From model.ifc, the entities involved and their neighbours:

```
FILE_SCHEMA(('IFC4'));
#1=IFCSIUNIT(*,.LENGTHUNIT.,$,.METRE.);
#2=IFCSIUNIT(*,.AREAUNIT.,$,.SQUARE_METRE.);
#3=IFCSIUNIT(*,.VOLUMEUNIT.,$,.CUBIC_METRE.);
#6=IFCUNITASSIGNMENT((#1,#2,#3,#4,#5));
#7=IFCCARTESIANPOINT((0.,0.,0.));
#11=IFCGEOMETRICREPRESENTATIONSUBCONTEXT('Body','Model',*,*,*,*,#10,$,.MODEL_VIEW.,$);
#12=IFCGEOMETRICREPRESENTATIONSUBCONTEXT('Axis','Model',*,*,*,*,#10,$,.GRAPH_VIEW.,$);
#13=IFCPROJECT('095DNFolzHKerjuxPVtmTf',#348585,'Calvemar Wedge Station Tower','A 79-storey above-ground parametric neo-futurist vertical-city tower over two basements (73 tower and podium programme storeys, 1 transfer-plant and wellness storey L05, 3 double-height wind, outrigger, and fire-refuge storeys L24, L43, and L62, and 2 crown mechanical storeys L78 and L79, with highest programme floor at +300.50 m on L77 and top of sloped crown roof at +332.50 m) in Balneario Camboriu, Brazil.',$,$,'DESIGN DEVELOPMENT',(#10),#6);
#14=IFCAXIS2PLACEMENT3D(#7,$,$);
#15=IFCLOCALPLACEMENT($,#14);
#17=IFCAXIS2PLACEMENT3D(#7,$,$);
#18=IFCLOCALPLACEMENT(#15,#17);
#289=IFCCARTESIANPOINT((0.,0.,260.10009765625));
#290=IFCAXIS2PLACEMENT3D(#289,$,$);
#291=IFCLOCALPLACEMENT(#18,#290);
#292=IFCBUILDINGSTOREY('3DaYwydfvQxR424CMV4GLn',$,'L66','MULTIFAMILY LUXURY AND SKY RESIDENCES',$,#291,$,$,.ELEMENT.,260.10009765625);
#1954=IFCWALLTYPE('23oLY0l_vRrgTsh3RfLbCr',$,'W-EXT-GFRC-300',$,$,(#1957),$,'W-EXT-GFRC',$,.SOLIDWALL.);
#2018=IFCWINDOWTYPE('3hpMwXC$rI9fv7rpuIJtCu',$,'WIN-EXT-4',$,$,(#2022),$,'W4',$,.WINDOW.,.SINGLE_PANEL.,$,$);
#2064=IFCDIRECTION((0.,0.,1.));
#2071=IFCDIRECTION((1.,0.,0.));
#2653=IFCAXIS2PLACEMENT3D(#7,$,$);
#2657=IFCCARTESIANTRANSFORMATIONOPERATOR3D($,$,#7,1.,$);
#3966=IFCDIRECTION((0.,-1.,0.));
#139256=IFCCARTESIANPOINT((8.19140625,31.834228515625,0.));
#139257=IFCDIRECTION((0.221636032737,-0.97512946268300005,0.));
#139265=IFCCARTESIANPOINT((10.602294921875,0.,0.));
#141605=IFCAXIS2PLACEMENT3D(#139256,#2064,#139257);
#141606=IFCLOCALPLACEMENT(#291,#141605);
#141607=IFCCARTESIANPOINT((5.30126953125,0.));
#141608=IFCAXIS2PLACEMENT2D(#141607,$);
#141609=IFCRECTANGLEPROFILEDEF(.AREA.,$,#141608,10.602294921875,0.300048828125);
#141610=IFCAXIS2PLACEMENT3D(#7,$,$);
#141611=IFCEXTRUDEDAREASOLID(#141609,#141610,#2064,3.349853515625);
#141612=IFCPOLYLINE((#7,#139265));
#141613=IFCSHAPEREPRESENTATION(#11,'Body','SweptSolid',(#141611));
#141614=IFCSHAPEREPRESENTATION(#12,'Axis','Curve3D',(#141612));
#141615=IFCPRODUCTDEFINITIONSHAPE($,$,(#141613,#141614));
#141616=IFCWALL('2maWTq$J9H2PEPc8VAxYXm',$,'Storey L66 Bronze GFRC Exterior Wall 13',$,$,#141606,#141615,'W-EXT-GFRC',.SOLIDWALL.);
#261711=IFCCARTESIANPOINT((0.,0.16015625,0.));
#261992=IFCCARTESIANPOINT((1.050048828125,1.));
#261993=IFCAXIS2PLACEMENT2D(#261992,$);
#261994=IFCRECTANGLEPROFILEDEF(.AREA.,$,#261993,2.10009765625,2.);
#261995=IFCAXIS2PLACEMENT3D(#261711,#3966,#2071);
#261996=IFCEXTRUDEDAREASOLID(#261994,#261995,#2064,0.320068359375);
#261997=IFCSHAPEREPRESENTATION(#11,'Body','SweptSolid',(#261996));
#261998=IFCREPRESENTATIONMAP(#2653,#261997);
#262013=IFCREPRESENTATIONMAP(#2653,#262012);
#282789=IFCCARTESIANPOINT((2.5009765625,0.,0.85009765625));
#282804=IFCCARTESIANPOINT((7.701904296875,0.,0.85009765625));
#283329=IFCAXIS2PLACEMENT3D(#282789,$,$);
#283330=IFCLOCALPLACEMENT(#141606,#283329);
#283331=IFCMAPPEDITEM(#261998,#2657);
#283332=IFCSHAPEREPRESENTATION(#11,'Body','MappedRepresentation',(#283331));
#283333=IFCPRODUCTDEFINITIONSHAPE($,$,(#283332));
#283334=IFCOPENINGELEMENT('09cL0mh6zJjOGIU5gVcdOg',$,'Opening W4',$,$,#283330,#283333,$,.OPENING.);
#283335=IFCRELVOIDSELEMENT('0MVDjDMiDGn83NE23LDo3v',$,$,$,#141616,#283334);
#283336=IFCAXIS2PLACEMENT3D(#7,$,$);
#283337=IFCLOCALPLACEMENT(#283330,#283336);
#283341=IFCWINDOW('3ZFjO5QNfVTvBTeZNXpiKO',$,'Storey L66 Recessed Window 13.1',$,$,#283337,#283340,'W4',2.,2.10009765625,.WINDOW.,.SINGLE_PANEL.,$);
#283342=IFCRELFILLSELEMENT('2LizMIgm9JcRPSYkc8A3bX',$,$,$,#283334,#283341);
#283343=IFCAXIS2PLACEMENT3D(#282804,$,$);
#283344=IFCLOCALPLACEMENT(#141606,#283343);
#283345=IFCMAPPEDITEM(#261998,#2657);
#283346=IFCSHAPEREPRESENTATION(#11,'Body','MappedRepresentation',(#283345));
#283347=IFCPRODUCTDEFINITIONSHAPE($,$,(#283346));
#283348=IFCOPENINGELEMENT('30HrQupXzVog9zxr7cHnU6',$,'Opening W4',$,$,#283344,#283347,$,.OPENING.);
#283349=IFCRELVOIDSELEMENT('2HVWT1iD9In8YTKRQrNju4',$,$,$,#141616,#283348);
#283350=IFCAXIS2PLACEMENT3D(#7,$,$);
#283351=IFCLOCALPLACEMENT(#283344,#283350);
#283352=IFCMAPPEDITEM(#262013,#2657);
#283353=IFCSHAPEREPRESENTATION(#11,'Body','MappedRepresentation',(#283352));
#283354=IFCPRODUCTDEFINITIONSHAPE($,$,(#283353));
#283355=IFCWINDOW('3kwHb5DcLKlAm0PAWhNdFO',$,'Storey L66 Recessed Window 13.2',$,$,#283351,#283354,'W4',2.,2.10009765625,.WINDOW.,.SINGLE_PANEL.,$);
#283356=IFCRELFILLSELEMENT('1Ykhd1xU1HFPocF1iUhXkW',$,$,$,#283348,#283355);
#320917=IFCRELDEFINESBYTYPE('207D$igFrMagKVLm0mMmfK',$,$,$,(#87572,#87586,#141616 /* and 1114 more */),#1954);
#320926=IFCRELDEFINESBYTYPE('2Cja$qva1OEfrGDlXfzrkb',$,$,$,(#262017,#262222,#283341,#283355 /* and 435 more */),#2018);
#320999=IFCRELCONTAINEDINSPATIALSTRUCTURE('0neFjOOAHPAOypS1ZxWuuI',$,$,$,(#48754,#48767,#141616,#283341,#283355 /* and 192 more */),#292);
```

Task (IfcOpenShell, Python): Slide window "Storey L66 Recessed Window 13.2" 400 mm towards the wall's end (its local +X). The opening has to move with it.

```python
import ifcopenshell
import ifcopenshell.api.geometry
import ifcopenshell.util.placement

model = ifcopenshell.open("model.ifc")

window = model.by_id(283355)
opening = window.FillsVoids[0].RelatingOpeningElement
wall = opening.VoidsElements[0].RelatingBuildingElement

wall_matrix = ifcopenshell.util.placement.get_local_placement(wall.ObjectPlacement)
shift = wall_matrix[:3, 0] * 0.4
before = ifcopenshell.util.placement.get_local_placement(window.ObjectPlacement)[:3, 3].copy()

# The window is placed relative to its opening, so it follows when the opening moves.
matrix = ifcopenshell.util.placement.get_local_placement(opening.ObjectPlacement)
matrix[:3, 3] += shift
ifcopenshell.api.geometry.edit_object_placement(
    model, product=opening, matrix=matrix, is_si=False, should_transform_children=True
)

after = ifcopenshell.util.placement.get_local_placement(window.ObjectPlacement)[:3, 3]
print("window moved by", (after - before).round(3) + 0.0)

model.write("model_edited.ifc")
```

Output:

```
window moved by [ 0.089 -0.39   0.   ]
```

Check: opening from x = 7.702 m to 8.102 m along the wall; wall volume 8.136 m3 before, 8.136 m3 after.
